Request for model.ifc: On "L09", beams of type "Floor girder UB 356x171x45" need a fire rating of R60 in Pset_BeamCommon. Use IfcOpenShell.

First a look at what the model holds.

```python
import ifcopenshell
import ifcopenshell.util.element

model = ifcopenshell.open("model.ifc")
print(model.schema)
storey = next(s for s in model.by_type("IfcBuildingStorey") if s.Name == "L09")
beams = [e for e in ifcopenshell.util.element.get_decomposition(storey) if e.is_a("IfcBeam")]
seen = {}
for e in beams:
    element_type = ifcopenshell.util.element.get_type(e)
    key = (element_type.Name if element_type != e and element_type else None, ifcopenshell.util.element.get_pset(e, "Pset_BeamCommon", "FireRating"))
    seen[key] = seen.get(key, 0) + 1
for (name, value), count in sorted(seen.items(), key=str):
    print(count, "x", name, "|", value)
```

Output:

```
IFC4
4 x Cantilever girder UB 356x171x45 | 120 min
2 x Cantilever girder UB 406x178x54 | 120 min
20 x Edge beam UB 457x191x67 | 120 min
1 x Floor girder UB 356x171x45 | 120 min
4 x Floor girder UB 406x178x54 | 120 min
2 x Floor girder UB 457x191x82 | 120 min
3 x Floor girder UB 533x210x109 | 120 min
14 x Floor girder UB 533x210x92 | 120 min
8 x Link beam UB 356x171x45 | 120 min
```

```python
import ifcopenshell
import ifcopenshell.api.pset
import ifcopenshell.util.element

model = ifcopenshell.open("model.ifc")

storey = next(s for s in model.by_type("IfcBuildingStorey") if s.Name == "L09")
beams = [e for e in ifcopenshell.util.element.get_decomposition(storey) if e.is_a("IfcBeam")]

count = 0
for e in beams:
    element_type = ifcopenshell.util.element.get_type(e)
    if element_type in (None, e) or element_type.Name != "Floor girder UB 356x171x45":
        continue
    found = ifcopenshell.util.element.get_pset(e, "Pset_BeamCommon", should_inherit=False)
    if found:
        pset = model.by_id(found["id"])
        if len(ifcopenshell.util.element.get_elements_by_pset(pset)) > 1:
            pset = ifcopenshell.api.pset.unshare_pset(model, products=[e], pset=pset)[0]
    else:
        pset = ifcopenshell.api.pset.add_pset(model, product=e, name="Pset_BeamCommon")
    ifcopenshell.api.pset.edit_pset(model, pset=pset, properties={"FireRating": "R60"})
    count += 1

print(count, "beams updated")

model.write("model_v2.ifc")
```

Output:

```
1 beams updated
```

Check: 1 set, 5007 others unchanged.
